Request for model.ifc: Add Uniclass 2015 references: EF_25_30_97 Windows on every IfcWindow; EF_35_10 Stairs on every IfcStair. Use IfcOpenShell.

First a look at what the model holds.

```python
import ifcopenshell

model = ifcopenshell.open("model.ifc")
print(model.schema)
print("classifications:", [c.Name for c in model.by_type("IfcClassification")])
for ifc_class in ("IfcDoor", "IfcRoof", "IfcStair", "IfcWall", "IfcWindow"):
    print(ifc_class, len(model.by_type(ifc_class)))
```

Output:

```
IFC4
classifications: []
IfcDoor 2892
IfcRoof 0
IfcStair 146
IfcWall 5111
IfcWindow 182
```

```python
import ifcopenshell
import ifcopenshell.api.classification

model = ifcopenshell.open("model.ifc")

system = ifcopenshell.api.classification.add_classification(model, classification="Uniclass 2015")

codes = {
    "IfcWindow": ("EF_25_30_97", "Windows"),
    "IfcStair": ("EF_35_10", "Stairs"),
}
for ifc_class, (code, name) in codes.items():
    products = model.by_type(ifc_class)
    ifcopenshell.api.classification.add_reference(
        model, products=products, classification=system, identification=code, name=name
    )
    print(code, len(products))

model.write("model_rev.ifc")
```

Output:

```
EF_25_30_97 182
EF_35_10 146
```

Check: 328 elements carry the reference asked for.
